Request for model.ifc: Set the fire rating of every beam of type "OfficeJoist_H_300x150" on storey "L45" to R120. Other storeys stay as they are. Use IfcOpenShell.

First a look at what the model holds.

```python
import ifcopenshell
import ifcopenshell.util.element

model = ifcopenshell.open("model.ifc")
print(model.schema)
storey = next(s for s in model.by_type("IfcBuildingStorey") if s.Name == "L45")
beams = [e for e in ifcopenshell.util.element.get_decomposition(storey) if e.is_a("IfcBeam")]
seen = {}
for e in beams:
    element_type = ifcopenshell.util.element.get_type(e)
    key = (element_type.Name if element_type != e and element_type else None, ifcopenshell.util.element.get_pset(e, "Pset_BeamCommon", "FireRating"))
    seen[key] = seen.get(key, 0) + 1
for (name, value), count in sorted(seen.items(), key=str):
    print(count, "x", name, "|", value)
```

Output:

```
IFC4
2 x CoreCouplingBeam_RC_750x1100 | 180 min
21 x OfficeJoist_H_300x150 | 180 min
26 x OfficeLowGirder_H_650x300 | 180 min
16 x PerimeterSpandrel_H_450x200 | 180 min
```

```python
import ifcopenshell
import ifcopenshell.api.pset
import ifcopenshell.util.element

model = ifcopenshell.open("model.ifc")

storey = next(s for s in model.by_type("IfcBuildingStorey") if s.Name == "L45")
beams = [e for e in ifcopenshell.util.element.get_decomposition(storey) if e.is_a("IfcBeam")]

count = 0
for e in beams:
    element_type = ifcopenshell.util.element.get_type(e)
    if element_type in (None, e) or element_type.Name != "OfficeJoist_H_300x150":
        continue
    # add_pset returns the element's existing set when there is one.
    pset = ifcopenshell.api.pset.add_pset(model, product=e, name="Pset_BeamCommon")
    ifcopenshell.api.pset.edit_pset(model, pset=pset, properties={"FireRating": "R120"})
    count += 1

print(count, "beams updated")

model.write("model_v2.ifc")
```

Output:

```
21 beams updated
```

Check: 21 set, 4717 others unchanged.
